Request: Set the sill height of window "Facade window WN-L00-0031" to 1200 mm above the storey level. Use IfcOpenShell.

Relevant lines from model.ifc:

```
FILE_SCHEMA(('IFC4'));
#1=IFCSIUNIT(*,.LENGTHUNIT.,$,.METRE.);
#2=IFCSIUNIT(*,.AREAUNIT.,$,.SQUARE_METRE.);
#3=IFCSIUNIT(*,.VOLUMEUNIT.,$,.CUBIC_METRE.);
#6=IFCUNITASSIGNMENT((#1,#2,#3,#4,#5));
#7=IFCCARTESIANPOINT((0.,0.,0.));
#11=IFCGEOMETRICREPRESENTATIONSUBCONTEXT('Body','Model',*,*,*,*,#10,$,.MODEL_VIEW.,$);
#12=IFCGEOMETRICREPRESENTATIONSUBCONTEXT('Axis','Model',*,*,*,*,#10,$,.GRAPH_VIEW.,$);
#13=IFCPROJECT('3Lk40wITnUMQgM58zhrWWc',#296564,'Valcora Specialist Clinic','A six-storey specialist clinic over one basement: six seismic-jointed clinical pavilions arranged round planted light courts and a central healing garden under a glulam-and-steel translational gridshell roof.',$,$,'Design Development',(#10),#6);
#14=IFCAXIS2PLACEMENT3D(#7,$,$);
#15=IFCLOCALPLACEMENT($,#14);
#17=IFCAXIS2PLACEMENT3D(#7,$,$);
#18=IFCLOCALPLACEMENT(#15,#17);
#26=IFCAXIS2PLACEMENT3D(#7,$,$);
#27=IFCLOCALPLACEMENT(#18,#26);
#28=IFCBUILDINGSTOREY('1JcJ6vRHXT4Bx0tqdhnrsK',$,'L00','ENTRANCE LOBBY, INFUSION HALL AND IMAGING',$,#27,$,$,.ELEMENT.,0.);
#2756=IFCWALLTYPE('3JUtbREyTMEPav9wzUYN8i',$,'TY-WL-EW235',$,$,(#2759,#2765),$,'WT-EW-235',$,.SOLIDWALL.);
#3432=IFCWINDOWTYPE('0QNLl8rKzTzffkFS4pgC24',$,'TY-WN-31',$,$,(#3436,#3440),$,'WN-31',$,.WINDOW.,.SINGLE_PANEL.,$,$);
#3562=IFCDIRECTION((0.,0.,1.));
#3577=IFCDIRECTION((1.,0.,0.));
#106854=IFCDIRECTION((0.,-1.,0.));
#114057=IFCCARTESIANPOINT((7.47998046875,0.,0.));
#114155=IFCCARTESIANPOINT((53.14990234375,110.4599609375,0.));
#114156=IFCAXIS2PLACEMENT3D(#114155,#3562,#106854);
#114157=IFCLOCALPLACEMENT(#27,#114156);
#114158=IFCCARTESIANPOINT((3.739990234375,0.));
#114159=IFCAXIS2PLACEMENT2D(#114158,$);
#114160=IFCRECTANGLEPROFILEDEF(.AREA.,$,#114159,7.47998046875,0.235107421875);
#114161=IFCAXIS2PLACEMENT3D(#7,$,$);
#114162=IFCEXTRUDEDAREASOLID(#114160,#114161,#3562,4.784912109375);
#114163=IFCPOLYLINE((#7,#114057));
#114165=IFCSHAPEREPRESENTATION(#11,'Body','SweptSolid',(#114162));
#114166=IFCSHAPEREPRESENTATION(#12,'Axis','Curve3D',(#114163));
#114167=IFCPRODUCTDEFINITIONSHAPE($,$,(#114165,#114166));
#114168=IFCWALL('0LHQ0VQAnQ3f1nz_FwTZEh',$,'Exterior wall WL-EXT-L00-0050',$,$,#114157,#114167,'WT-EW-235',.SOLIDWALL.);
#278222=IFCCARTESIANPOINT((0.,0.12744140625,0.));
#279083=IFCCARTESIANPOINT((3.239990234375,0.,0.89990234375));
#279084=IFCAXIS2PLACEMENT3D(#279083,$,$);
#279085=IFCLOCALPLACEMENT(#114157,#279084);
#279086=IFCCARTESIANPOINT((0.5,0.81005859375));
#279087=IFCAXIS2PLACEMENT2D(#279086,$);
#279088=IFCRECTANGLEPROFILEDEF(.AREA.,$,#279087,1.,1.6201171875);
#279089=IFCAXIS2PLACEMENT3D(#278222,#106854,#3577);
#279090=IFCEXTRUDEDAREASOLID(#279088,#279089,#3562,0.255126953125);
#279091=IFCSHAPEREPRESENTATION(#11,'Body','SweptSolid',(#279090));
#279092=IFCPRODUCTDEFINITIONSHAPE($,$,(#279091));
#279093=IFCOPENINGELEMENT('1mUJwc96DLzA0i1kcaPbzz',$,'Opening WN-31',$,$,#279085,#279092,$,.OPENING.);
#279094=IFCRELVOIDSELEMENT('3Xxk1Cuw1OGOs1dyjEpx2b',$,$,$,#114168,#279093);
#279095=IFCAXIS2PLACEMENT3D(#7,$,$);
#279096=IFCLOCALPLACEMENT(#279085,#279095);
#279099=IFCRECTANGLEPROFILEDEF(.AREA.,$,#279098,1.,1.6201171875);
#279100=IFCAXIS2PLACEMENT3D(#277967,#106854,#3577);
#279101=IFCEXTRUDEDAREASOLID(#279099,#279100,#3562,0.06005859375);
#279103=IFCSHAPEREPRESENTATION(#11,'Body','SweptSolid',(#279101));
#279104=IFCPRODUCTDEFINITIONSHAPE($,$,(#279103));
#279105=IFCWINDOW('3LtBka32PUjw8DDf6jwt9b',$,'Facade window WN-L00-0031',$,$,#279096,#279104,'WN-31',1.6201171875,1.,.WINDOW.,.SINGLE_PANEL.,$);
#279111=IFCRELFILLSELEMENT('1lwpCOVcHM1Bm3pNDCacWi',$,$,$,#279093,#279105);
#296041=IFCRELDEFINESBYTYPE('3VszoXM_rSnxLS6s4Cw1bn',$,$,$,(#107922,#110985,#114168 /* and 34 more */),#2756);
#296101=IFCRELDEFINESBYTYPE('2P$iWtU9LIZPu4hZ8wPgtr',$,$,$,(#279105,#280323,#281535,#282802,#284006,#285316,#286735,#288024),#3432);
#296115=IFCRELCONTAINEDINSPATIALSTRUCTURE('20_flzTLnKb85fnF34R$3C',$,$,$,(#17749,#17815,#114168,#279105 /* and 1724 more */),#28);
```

```python
import numpy as np
import ifcopenshell
import ifcopenshell.api.geometry
import ifcopenshell.geom
import ifcopenshell.util.element
import ifcopenshell.util.placement
import ifcopenshell.util.shape
import ifcopenshell.util.unit

model = ifcopenshell.open("model.ifc")
unit_scale = ifcopenshell.util.unit.calculate_unit_scale(model)

window = model.by_guid("3LtBka32PUjw8DDf6jwt9b")
opening = window.FillsVoids[0].RelatingOpeningElement
storey = ifcopenshell.util.element.get_container(window, ifc_class="IfcBuildingStorey")
level = ifcopenshell.util.placement.get_local_placement(storey.ObjectPlacement)[2, 3]

# The opening's origin need not be at the sill, so measure its lowest point.
shape = ifcopenshell.geom.create_shape(ifcopenshell.geom.settings(), opening)
bottom = ifcopenshell.util.shape.get_shape_bottom_elevation(shape, shape.geometry) / unit_scale
dz = level + 1.2 / unit_scale - bottom

shift = np.array([0.0, 0.0, dz])
# The window is placed relative to its opening, so it follows when the opening moves.
matrix = ifcopenshell.util.placement.get_local_placement(opening.ObjectPlacement)
matrix[:3, 3] += shift
ifcopenshell.api.geometry.edit_object_placement(
    model, product=opening, matrix=matrix, is_si=False, should_transform_children=True
)

print(f"moved by {dz * unit_scale:+.3f} m")

model.write("model_v2.ifc")
```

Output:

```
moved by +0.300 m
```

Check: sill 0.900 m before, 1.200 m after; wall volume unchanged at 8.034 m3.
